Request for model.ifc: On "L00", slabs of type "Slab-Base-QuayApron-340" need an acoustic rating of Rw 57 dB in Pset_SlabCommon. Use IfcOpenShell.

First a look at what the model holds.

```python
import ifcopenshell
import ifcopenshell.util.element

model = ifcopenshell.open("model.ifc")
print(model.schema)
storey = next(s for s in model.by_type("IfcBuildingStorey") if s.Name == "L00")
slabs = [e for e in ifcopenshell.util.element.get_decomposition(storey) if e.is_a("IfcSlab")]
seen = {}
for e in slabs:
    element_type = ifcopenshell.util.element.get_type(e)
    key = (element_type.Name if element_type != e and element_type else None, ifcopenshell.util.element.get_pset(e, "Pset_SlabCommon", "AcousticRating"))
    seen[key] = seen.get(key, 0) + 1
for (name, value), count in sorted(seen.items(), key=str):
    print(count, "x", name, "|", value)
```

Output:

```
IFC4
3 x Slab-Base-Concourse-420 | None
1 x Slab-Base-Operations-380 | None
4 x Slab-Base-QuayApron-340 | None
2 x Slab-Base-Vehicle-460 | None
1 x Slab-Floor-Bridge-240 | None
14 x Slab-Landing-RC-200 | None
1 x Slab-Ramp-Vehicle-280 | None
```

```python
import ifcopenshell
import ifcopenshell.api.pset
import ifcopenshell.util.element

model = ifcopenshell.open("model.ifc")

storey = next(s for s in model.by_type("IfcBuildingStorey") if s.Name == "L00")
slabs = [e for e in ifcopenshell.util.element.get_decomposition(storey) if e.is_a("IfcSlab")]

count = 0
for e in slabs:
    element_type = ifcopenshell.util.element.get_type(e)
    if element_type in (None, e) or element_type.Name != "Slab-Base-QuayApron-340":
        continue
    # add_pset returns the element's existing set when there is one.
    pset = ifcopenshell.api.pset.add_pset(model, product=e, name="Pset_SlabCommon")
    ifcopenshell.api.pset.edit_pset(model, pset=pset, properties={"AcousticRating": "Rw 57 dB"})
    count += 1

print(count, "slabs updated")

model.write("model-out.ifc")
```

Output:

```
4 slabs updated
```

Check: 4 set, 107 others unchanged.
